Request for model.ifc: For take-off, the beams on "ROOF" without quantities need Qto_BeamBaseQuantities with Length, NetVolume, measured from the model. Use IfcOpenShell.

First a look at what the model holds.

```python
import ifcopenshell
import ifcopenshell.util.element
import ifcopenshell.util.unit

model = ifcopenshell.open("model.ifc")
print(model.schema)
for unit_type in ("LENGTHUNIT", "AREAUNIT", "VOLUMEUNIT"):
    print(unit_type, ifcopenshell.util.unit.calculate_unit_scale(model, unit_type))
storey = next(s for s in model.by_type("IfcBuildingStorey") if s.Name == "ROOF")
beams = [e for e in ifcopenshell.util.element.get_decomposition(storey) if e.is_a("IfcBeam")]
for e in sorted(beams, key=lambda e: e.id()):
    print(e.id(), e.is_a(), e.Name, list(ifcopenshell.util.element.get_psets(e, qtos_only=True)), sep=" | ")
```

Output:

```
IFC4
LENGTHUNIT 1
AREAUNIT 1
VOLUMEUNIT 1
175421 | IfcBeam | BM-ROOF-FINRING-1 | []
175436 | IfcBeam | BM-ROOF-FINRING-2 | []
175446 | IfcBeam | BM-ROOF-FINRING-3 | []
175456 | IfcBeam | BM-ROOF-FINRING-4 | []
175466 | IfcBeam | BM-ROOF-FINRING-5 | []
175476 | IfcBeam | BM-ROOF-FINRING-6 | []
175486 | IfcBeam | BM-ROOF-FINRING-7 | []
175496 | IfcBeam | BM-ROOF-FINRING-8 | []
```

```python
import ifcopenshell
import ifcopenshell.api.pset
import ifcopenshell.geom
import ifcopenshell.util.element
import ifcopenshell.util.shape
import ifcopenshell.util.unit

model = ifcopenshell.open("model.ifc")
unit_scale = ifcopenshell.util.unit.calculate_unit_scale(model)
volume_scale = ifcopenshell.util.unit.calculate_unit_scale(model, "VOLUMEUNIT")
settings = ifcopenshell.geom.settings()

storey = next(s for s in model.by_type("IfcBuildingStorey") if s.Name == "ROOF")
beams = [e for e in ifcopenshell.util.element.get_decomposition(storey) if e.is_a("IfcBeam")]

for e in sorted(beams, key=lambda e: e.id()):
    if ifcopenshell.util.element.get_psets(e, qtos_only=True, should_inherit=False):
        continue
    # Geometry comes back in metres, in the element's own axes.
    shape = ifcopenshell.geom.create_shape(settings, e)
    values = {
        "Length": ifcopenshell.util.shape.get_max_xyz(shape.geometry) / unit_scale,
        "NetVolume": ifcopenshell.util.shape.get_volume(shape.geometry) / volume_scale,
    }
    qto = ifcopenshell.api.pset.add_qto(model, product=e, name="Qto_BeamBaseQuantities")
    ifcopenshell.api.pset.edit_qto(model, qto=qto, properties=values)
    print(e.id(), {k: round(v, 3) for k, v in values.items()})

model.write("model_rev.ifc")
```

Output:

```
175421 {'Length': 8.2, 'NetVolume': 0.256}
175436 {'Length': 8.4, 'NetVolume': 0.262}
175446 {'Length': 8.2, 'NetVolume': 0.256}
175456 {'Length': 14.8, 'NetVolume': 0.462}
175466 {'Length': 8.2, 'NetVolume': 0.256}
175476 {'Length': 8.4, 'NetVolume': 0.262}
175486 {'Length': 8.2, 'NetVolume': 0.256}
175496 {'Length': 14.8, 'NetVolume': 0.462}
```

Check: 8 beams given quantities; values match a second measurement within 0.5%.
